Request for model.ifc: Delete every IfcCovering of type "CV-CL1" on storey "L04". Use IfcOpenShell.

First a look at what the model holds.

```python
import ifcopenshell
import ifcopenshell.util.element

model = ifcopenshell.open("model.ifc")
print(model.schema)
storey = next(s for s in model.by_type("IfcBuildingStorey") if s.Name == "L04")
coverings = [e for e in ifcopenshell.util.element.get_decomposition(storey) if e.is_a("IfcCovering")]
seen = {}
for e in coverings:
    element_type = ifcopenshell.util.element.get_type(e)
    name = element_type.Name if element_type not in (None, e) else None
    seen[name] = seen.get(name, 0) + 1
for name, count in sorted(seen.items(), key=str):
    print(count, "x", name)
```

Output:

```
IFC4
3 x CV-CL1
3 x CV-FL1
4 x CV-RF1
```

```python
import ifcopenshell
import ifcopenshell.api.root
import ifcopenshell.util.element

model = ifcopenshell.open("model.ifc")

storey = next(s for s in model.by_type("IfcBuildingStorey") if s.Name == "L04")
coverings = [e for e in ifcopenshell.util.element.get_decomposition(storey) if e.is_a("IfcCovering")]
targets = [e for e in coverings if (t := ifcopenshell.util.element.get_type(e)) not in (None, e) and t.Name == "CV-CL1"]

for e in targets:
    ifcopenshell.api.root.remove_product(model, product=e)
print(len(targets), "removed")

model.write("model_v2.ifc")
```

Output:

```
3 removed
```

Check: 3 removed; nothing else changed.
